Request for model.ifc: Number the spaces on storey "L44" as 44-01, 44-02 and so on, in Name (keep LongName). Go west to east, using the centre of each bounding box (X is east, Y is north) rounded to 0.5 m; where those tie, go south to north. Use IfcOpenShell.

First a look at what the model holds.

```python
import ifcopenshell
import ifcopenshell.util.element
import ifcopenshell.util.placement

model = ifcopenshell.open("model.ifc")
print(model.schema)
storey = next(s for s in model.by_type("IfcBuildingStorey") if s.Name == "L44")
spaces = [e for e in ifcopenshell.util.element.get_decomposition(storey) if e.is_a("IfcSpace")]
for e in sorted(spaces, key=lambda e: e.id()):
    origin = ifcopenshell.util.placement.get_local_placement(e.ObjectPlacement)[:3, 3]
    print(e.id(), e.Name, e.LongName, origin.round(2) + 0.0, sep=" | ")
```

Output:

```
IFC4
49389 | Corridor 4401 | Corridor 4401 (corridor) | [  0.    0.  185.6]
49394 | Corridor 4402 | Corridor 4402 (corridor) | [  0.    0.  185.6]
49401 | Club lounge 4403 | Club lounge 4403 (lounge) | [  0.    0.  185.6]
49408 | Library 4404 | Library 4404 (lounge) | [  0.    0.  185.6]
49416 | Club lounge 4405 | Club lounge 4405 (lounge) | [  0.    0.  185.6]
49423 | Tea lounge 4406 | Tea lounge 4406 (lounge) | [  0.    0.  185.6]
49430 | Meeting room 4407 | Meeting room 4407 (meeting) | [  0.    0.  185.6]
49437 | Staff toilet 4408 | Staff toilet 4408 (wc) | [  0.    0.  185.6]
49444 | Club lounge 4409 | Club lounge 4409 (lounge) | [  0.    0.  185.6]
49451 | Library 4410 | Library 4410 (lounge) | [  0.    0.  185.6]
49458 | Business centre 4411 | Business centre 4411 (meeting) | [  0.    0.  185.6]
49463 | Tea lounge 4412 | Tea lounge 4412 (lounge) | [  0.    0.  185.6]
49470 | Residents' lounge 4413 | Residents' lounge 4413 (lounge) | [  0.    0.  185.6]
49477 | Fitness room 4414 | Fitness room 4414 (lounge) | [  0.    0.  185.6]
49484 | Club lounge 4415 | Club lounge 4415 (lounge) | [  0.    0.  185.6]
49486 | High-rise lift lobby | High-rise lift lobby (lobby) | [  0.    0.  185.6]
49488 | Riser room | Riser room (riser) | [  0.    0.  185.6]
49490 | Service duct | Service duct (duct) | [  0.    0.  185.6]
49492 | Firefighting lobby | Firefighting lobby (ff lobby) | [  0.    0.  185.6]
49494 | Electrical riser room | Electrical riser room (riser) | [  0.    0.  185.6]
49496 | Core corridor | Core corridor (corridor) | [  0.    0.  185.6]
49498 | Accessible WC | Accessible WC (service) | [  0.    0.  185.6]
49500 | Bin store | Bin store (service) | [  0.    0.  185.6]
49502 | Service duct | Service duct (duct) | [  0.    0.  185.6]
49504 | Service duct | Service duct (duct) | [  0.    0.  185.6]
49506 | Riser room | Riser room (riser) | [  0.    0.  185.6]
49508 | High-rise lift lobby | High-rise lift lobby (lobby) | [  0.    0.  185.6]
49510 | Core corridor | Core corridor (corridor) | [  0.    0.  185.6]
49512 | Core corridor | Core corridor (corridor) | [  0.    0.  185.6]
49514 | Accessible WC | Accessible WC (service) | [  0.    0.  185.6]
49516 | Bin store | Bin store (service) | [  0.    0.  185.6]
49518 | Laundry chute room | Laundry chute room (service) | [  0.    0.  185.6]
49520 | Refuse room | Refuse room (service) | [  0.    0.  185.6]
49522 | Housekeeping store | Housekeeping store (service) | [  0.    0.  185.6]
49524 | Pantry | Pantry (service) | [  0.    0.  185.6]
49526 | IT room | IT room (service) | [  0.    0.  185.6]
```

```python
import ifcopenshell
import ifcopenshell.geom
import ifcopenshell.util.element
import ifcopenshell.util.shape

model = ifcopenshell.open("model.ifc")
settings = ifcopenshell.geom.settings()
settings.set("use-world-coords", True)


def centre(element):
    shape = ifcopenshell.geom.create_shape(settings, element)
    return ifcopenshell.util.shape.get_bbox_centroid(shape.geometry)


storey = next(s for s in model.by_type("IfcBuildingStorey") if s.Name == "L44")
spaces = [e for e in ifcopenshell.util.element.get_decomposition(storey) if e.is_a("IfcSpace")]

# Insertion points can sit at a corner or the storey origin, so sort by the geometry (in metres).
centres = {e: centre(e) for e in spaces}
spaces.sort(key=lambda e: (round(centres[e][0] / 0.5), centres[e][1]))

for i, e in enumerate(spaces, start=1):
    number = f"44-{i:02d}"
    e.Name = number
    print(e.id(), number)

model.write("model-out.ifc")
```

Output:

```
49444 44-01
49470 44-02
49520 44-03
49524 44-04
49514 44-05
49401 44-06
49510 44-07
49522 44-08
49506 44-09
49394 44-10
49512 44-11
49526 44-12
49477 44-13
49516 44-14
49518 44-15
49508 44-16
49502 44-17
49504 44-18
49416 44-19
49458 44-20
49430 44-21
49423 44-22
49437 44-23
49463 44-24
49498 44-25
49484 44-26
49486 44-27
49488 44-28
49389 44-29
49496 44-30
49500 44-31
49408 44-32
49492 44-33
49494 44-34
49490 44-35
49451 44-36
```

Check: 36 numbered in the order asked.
